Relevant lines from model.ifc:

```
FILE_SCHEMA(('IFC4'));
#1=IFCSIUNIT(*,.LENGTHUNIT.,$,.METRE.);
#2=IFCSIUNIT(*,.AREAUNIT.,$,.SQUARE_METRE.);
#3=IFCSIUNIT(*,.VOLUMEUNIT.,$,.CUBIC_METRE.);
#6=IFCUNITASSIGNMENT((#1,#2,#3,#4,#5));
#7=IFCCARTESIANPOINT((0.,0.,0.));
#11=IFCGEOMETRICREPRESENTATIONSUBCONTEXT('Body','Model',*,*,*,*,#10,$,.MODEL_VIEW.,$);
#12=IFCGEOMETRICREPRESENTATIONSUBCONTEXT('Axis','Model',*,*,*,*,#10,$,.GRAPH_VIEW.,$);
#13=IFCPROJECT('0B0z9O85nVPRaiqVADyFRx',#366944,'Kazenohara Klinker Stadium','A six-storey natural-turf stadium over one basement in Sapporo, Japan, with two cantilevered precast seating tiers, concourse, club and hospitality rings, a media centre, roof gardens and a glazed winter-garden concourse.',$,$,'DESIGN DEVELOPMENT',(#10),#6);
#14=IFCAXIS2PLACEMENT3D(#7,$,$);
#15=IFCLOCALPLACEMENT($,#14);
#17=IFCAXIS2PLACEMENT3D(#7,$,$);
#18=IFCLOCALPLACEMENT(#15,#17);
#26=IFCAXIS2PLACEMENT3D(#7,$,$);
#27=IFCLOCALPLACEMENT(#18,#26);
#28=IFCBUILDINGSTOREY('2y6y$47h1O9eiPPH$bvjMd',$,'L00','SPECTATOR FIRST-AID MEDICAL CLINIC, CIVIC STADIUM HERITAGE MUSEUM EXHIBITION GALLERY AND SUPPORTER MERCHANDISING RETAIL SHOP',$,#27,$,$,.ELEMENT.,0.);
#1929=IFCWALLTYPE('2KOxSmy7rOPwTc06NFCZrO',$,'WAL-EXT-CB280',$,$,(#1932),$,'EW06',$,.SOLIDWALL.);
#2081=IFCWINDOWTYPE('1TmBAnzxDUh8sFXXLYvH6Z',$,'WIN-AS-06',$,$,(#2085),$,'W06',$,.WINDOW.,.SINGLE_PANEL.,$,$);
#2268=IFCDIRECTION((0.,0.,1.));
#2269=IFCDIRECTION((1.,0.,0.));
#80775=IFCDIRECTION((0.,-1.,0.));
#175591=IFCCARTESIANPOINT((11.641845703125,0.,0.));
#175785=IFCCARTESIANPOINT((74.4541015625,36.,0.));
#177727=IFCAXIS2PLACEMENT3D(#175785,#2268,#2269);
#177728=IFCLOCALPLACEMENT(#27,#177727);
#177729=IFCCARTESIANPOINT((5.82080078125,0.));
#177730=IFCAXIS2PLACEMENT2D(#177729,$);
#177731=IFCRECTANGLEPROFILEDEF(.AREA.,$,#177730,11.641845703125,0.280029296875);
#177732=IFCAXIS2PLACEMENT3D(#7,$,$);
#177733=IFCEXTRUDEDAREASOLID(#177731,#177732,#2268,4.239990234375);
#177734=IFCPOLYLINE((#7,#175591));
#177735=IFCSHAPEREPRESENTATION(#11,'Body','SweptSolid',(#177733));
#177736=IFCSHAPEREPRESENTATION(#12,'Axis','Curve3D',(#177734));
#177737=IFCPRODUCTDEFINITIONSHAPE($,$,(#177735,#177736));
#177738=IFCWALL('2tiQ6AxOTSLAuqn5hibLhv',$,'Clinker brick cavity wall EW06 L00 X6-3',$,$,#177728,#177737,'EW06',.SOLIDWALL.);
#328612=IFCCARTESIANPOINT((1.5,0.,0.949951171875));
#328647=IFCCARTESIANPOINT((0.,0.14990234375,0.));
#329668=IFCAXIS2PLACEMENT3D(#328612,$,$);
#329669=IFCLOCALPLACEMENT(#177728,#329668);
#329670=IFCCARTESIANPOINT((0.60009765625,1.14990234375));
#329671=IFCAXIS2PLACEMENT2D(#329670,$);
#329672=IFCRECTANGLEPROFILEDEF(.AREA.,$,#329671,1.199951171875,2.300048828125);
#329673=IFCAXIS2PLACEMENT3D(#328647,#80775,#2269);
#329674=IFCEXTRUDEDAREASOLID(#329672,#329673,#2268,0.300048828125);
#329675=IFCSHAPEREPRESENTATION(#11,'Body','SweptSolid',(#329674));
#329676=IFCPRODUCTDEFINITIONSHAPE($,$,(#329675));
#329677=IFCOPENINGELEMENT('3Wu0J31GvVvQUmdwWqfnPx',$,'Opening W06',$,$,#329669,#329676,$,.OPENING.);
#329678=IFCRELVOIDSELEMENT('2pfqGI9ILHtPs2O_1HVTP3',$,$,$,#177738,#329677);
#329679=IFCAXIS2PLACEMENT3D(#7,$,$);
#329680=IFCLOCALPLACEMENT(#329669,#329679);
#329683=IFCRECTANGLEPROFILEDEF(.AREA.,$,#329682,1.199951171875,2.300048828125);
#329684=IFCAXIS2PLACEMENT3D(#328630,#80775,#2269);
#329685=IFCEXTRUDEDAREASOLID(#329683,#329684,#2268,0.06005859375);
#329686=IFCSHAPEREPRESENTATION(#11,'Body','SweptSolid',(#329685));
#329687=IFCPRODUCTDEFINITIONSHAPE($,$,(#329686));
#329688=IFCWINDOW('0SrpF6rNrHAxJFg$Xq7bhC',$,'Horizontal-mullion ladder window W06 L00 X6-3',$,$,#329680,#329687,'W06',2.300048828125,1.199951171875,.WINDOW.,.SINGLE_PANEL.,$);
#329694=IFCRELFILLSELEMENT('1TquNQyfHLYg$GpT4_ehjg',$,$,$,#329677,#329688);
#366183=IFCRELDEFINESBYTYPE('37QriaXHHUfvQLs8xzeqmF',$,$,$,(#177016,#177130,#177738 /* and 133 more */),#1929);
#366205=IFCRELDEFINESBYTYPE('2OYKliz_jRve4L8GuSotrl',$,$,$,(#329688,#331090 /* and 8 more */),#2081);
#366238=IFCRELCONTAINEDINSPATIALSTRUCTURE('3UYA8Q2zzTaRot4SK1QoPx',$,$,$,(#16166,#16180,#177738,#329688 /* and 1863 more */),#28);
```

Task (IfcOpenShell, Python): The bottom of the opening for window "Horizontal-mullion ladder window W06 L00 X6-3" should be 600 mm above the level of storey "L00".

```python
import numpy as np
import ifcopenshell
import ifcopenshell.api.geometry
import ifcopenshell.geom
import ifcopenshell.util.element
import ifcopenshell.util.placement
import ifcopenshell.util.shape
import ifcopenshell.util.unit

model = ifcopenshell.open("model.ifc")
unit_scale = ifcopenshell.util.unit.calculate_unit_scale(model)

window = model.by_guid("0SrpF6rNrHAxJFg$Xq7bhC")
opening = window.FillsVoids[0].RelatingOpeningElement
storey = ifcopenshell.util.element.get_container(window, ifc_class="IfcBuildingStorey")
level = ifcopenshell.util.placement.get_local_placement(storey.ObjectPlacement)[2, 3]

# The opening's origin need not be at the sill, so measure its lowest point.
shape = ifcopenshell.geom.create_shape(ifcopenshell.geom.settings(), opening)
bottom = ifcopenshell.util.shape.get_shape_bottom_elevation(shape, shape.geometry) / unit_scale
dz = level + 0.6 - bottom

shift = np.array([0.0, 0.0, dz])
# The window is placed relative to its opening, so it follows when the opening moves.
matrix = ifcopenshell.util.placement.get_local_placement(opening.ObjectPlacement)
matrix[:3, 3] += shift
ifcopenshell.api.geometry.edit_object_placement(
    model, product=opening, matrix=matrix, is_si=False, should_transform_children=True
)

print(f"moved by {dz * unit_scale:+.3f} m")

model.write("model_edited.ifc")
```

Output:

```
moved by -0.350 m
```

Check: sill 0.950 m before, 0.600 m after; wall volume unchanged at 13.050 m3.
